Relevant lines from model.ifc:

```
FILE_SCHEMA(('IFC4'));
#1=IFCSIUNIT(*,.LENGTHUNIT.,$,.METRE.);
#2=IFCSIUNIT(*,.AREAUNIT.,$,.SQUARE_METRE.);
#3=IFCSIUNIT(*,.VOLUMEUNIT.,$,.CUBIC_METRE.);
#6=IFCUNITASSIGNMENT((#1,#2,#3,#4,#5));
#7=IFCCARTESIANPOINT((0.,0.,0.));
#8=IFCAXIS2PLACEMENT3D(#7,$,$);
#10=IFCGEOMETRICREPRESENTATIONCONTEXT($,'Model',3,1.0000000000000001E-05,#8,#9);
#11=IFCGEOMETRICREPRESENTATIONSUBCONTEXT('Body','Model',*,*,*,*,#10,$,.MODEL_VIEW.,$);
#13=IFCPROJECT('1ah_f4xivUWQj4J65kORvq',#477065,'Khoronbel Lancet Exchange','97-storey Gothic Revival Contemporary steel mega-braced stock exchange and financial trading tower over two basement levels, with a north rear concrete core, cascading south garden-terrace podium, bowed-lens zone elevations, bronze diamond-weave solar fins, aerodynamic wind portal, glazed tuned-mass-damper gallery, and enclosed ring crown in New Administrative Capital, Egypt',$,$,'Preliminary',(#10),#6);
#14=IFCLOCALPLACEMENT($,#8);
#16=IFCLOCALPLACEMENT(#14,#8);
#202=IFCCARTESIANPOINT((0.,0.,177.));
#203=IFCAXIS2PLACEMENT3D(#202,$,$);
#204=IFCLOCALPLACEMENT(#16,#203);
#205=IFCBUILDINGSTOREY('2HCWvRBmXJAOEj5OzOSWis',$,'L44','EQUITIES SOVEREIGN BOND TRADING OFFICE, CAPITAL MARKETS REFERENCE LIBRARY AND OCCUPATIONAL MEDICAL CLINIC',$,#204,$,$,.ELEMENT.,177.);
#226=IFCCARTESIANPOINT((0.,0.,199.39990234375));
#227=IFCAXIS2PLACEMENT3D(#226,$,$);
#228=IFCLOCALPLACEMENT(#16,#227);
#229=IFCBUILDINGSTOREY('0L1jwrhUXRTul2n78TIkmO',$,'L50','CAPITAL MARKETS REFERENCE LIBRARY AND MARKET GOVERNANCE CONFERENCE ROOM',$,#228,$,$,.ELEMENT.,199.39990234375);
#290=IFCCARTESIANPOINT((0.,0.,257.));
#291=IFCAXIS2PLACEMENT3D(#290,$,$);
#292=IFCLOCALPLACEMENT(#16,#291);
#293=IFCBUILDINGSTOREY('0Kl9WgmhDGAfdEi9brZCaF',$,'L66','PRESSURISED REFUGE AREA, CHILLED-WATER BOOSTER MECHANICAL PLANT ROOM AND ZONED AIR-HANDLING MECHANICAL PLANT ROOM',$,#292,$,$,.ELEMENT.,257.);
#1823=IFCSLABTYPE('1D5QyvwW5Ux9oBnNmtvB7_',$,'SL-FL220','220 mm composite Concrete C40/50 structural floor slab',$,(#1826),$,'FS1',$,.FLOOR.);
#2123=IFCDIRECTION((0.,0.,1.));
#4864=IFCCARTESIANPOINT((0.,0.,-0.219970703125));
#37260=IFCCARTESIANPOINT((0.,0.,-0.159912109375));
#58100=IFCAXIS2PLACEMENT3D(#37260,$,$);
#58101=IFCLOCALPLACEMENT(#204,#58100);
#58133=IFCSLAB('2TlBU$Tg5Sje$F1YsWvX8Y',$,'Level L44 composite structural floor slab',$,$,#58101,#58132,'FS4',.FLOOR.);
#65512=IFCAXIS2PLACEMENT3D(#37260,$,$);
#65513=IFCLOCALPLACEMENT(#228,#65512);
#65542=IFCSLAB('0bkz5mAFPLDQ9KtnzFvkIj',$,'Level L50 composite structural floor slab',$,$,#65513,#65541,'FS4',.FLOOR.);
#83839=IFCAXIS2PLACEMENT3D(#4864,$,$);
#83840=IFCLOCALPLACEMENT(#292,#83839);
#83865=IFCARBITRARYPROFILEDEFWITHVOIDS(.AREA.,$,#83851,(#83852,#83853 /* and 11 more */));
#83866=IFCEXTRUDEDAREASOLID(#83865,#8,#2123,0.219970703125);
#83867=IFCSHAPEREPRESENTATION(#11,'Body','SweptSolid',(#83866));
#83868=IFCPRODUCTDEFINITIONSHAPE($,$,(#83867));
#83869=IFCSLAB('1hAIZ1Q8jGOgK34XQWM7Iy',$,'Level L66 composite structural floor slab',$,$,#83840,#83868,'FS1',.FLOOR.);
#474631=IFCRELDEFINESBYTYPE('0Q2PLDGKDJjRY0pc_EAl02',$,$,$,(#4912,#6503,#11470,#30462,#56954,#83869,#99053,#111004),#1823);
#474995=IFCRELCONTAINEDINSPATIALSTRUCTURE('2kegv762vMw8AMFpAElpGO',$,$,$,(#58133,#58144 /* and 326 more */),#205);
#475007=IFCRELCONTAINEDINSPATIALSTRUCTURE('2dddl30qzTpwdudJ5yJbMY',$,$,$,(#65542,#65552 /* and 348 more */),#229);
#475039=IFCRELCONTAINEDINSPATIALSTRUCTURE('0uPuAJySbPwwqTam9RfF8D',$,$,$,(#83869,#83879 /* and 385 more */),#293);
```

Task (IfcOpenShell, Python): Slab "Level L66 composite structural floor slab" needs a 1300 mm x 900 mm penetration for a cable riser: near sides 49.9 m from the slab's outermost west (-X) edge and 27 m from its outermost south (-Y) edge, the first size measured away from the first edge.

```python
import numpy as np
import ifcopenshell
import ifcopenshell.api.feature
import ifcopenshell.api.geometry
import ifcopenshell.api.root
import ifcopenshell.geom
import ifcopenshell.util.placement
import ifcopenshell.util.representation
import ifcopenshell.util.shape
import ifcopenshell.util.unit

model = ifcopenshell.open("model.ifc")
unit_scale = ifcopenshell.util.unit.calculate_unit_scale(model)
settings = ifcopenshell.geom.settings()


def volume(element):
    """Net volume in cubic metres, openings subtracted."""
    shape = ifcopenshell.geom.create_shape(settings, element)
    return ifcopenshell.util.shape.get_volume(shape.geometry)


slab = model.by_guid("1hAIZ1Q8jGOgK34XQWM7Iy")
before = volume(slab)

# Extent in the slab's own axes, in metres. The edges named are its -X and -Y sides.
slab_shape = ifcopenshell.geom.create_shape(settings, slab)
vertices = ifcopenshell.util.shape.get_vertices(slab_shape.geometry)
x_min, y_min, bottom = vertices.min(axis=0)
top = vertices[:, 2].max()

opening = ifcopenshell.api.root.create_entity(model, ifc_class="IfcOpeningElement", name="Cable riser opening", predefined_type="OPENING")
context = ifcopenshell.util.representation.get_context(model, "Model", "Body", "MODEL_VIEW")
width, depth = 1.3, 0.9
outline = [(0.0, 0.0), (width, 0.0), (width, depth), (0.0, depth), (0.0, 0.0)]
# Overshoot both faces by 50 mm so the cut is clean.
shape = ifcopenshell.api.geometry.add_slab_representation(
    model, context=context, depth=top - bottom + 0.1, polyline=outline
)
ifcopenshell.api.geometry.assign_representation(model, product=opening, representation=shape)

matrix = ifcopenshell.util.placement.get_local_placement(slab.ObjectPlacement)
matrix[:, 3] = matrix @ np.append(np.array([x_min + 49.9, y_min + 27, bottom - 0.05]) / unit_scale, 1.0)
ifcopenshell.api.geometry.edit_object_placement(model, product=opening, matrix=matrix, is_si=False)
ifcopenshell.api.feature.add_feature(model, feature=opening, element=slab)

after = volume(slab)

print(f"slab volume {before:.3f} -> {after:.3f} m3")

model.write("model_v2.ifc")
```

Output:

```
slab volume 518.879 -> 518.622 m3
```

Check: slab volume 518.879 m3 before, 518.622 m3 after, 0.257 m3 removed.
